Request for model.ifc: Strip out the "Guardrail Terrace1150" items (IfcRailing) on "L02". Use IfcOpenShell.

First a look at what the model holds.

```python
import ifcopenshell
import ifcopenshell.util.element

model = ifcopenshell.open("model.ifc")
print(model.schema)
storey = next(s for s in model.by_type("IfcBuildingStorey") if s.Name == "L02")
railings = [e for e in ifcopenshell.util.element.get_decomposition(storey) if e.is_a("IfcRailing")]
seen = {}
for e in railings:
    element_type = ifcopenshell.util.element.get_type(e)
    name = element_type.Name if element_type not in (None, e) else None
    seen[name] = seen.get(name, 0) + 1
for name, count in sorted(seen.items(), key=str):
    print(count, "x", name)
```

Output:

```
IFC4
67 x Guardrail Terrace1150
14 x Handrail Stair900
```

```python
import ifcopenshell
import ifcopenshell.api.root
import ifcopenshell.util.element

model = ifcopenshell.open("model.ifc")

storey = next(s for s in model.by_type("IfcBuildingStorey") if s.Name == "L02")
railings = [e for e in ifcopenshell.util.element.get_decomposition(storey) if e.is_a("IfcRailing")]
targets = [e for e in railings if (t := ifcopenshell.util.element.get_type(e)) not in (None, e) and t.Name == "Guardrail Terrace1150"]

for e in targets:
    ifcopenshell.api.root.remove_product(model, product=e)
print(len(targets), "removed")

model.write("model_v2.ifc")
```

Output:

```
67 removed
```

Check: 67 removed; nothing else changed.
